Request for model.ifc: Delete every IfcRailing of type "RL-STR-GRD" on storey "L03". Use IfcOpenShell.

First a look at what the model holds.

```python
import ifcopenshell
import ifcopenshell.util.element

model = ifcopenshell.open("model.ifc")
print(model.schema)
storey = next(s for s in model.by_type("IfcBuildingStorey") if s.Name == "L03")
railings = [e for e in ifcopenshell.util.element.get_decomposition(storey) if e.is_a("IfcRailing")]
seen = {}
for e in railings:
    element_type = ifcopenshell.util.element.get_type(e)
    name = element_type.Name if element_type not in (None, e) else None
    seen[name] = seen.get(name, 0) + 1
for name, count in sorted(seen.items(), key=str):
    print(count, "x", name)
```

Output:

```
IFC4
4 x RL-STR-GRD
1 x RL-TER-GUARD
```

```python
import ifcopenshell
import ifcopenshell.api.root
import ifcopenshell.util.element

model = ifcopenshell.open("model.ifc")

storey = next(s for s in model.by_type("IfcBuildingStorey") if s.Name == "L03")
railings = [e for e in ifcopenshell.util.element.get_decomposition(storey) if e.is_a("IfcRailing")]
targets = [e for e in railings if (t := ifcopenshell.util.element.get_type(e)) not in (None, e) and t.Name == "RL-STR-GRD"]

for e in targets:
    ifcopenshell.api.root.remove_product(model, product=e)
print(len(targets), "removed")

model.write("model-out.ifc")
```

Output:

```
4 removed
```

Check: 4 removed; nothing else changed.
